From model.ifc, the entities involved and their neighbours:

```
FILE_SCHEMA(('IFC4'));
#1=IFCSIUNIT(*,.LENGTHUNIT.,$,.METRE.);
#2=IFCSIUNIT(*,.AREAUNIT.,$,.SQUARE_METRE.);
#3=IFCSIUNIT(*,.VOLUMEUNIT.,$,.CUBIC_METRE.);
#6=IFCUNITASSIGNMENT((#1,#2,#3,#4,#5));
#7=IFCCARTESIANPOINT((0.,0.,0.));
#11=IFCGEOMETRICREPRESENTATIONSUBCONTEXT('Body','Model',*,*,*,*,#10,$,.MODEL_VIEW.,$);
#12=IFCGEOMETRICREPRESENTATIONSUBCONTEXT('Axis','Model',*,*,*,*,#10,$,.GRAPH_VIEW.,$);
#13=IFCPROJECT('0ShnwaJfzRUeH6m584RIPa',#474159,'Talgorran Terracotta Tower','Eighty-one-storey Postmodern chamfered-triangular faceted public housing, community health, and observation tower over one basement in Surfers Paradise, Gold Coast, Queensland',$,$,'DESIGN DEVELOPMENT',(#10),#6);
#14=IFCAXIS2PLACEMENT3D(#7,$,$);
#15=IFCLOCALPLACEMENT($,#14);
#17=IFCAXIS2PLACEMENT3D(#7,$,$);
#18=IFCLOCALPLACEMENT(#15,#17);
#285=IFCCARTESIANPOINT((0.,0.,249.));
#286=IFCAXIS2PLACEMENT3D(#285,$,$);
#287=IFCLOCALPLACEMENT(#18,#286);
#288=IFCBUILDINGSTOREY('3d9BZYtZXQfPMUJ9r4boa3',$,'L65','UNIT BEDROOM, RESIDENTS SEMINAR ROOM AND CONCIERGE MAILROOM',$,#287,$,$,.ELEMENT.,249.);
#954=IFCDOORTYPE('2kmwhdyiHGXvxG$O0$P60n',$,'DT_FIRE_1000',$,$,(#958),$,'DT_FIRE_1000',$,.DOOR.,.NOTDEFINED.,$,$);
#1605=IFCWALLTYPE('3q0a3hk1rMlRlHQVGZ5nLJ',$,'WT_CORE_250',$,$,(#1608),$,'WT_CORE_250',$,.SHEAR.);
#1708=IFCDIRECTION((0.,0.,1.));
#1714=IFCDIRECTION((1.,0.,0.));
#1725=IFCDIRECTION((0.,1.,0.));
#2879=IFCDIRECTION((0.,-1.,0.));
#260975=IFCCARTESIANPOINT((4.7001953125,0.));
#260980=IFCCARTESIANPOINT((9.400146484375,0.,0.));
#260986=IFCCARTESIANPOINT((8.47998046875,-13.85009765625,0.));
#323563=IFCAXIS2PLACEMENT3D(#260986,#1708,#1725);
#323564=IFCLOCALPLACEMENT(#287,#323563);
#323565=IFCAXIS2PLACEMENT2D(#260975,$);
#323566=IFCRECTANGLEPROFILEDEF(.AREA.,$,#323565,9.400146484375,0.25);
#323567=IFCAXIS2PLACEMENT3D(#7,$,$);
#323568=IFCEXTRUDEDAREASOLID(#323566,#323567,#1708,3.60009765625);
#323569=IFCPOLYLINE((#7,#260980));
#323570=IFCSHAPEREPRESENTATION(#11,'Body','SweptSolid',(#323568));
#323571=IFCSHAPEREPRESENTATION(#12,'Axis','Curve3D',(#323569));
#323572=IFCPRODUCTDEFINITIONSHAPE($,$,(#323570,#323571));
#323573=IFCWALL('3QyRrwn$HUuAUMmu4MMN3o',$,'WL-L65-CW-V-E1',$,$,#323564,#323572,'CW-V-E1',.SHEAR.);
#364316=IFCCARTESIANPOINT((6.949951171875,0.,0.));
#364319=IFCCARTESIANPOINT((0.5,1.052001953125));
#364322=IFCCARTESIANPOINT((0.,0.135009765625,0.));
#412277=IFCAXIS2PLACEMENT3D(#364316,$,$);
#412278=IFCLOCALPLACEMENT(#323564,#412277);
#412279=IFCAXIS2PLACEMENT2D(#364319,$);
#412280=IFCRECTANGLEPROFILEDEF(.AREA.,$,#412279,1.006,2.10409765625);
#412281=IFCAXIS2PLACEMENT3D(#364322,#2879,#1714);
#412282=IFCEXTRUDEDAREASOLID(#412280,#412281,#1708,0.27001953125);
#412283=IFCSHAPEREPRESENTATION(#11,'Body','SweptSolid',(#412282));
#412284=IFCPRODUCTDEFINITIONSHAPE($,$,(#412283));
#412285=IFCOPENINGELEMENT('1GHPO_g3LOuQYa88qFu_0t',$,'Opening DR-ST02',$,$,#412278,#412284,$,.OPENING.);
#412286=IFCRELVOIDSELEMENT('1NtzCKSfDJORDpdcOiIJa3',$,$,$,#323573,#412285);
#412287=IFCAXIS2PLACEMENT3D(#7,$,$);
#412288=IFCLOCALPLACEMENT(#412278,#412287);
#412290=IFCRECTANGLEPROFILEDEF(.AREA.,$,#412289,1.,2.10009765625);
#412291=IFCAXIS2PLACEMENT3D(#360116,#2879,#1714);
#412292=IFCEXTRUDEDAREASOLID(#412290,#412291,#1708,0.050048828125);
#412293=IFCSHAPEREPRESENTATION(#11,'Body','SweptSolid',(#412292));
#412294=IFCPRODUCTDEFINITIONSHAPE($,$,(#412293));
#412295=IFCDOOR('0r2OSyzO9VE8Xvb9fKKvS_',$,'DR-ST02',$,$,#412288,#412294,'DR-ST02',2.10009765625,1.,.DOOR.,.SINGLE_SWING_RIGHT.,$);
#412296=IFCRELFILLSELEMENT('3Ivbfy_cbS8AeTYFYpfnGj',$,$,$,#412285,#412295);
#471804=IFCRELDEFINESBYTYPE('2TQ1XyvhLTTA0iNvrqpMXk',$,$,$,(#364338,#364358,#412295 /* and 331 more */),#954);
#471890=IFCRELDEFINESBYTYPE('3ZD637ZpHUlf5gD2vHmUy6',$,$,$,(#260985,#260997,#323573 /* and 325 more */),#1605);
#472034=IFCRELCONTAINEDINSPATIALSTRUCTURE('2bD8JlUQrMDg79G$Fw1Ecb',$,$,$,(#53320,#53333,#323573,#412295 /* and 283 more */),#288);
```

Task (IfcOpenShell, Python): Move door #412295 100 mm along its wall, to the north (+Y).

```python
import ifcopenshell
import ifcopenshell.api.geometry
import ifcopenshell.util.placement
import ifcopenshell.util.unit

model = ifcopenshell.open("model.ifc")
unit_scale = ifcopenshell.util.unit.calculate_unit_scale(model)

door = model.by_id(412295)
opening = door.FillsVoids[0].RelatingOpeningElement
wall = opening.VoidsElements[0].RelatingBuildingElement

wall_matrix = ifcopenshell.util.placement.get_local_placement(wall.ObjectPlacement)
shift = wall_matrix[:3, 0] * 0.1 / unit_scale
before = ifcopenshell.util.placement.get_local_placement(door.ObjectPlacement)[:3, 3].copy()

# The door is placed relative to its opening, so it follows when the opening moves.
matrix = ifcopenshell.util.placement.get_local_placement(opening.ObjectPlacement)
matrix[:3, 3] += shift
ifcopenshell.api.geometry.edit_object_placement(
    model, product=opening, matrix=matrix, is_si=False, should_transform_children=True
)

after = ifcopenshell.util.placement.get_local_placement(door.ObjectPlacement)[:3, 3]
print("door moved by", (after - before).round(3) + 0.0)

model.write("model_edited.ifc")
```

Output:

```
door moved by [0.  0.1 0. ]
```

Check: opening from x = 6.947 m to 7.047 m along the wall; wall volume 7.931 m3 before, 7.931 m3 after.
